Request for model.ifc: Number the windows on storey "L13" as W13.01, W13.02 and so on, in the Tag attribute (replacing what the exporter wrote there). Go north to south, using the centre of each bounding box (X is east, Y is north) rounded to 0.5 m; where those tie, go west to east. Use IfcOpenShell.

First a look at what the model holds.

```python
import ifcopenshell
import ifcopenshell.util.element
import ifcopenshell.util.placement

model = ifcopenshell.open("model.ifc")
print(model.schema)
storey = next(s for s in model.by_type("IfcBuildingStorey") if s.Name == "L13")
windows = [e for e in ifcopenshell.util.element.get_decomposition(storey) if e.is_a("IfcWindow")]
for e in sorted(windows, key=lambda e: e.id()):
    origin = ifcopenshell.util.placement.get_local_placement(e.ObjectPlacement)[:3, 3]
    print(e.id(), e.Tag, e.Name, origin.round(2) + 0.0, sep=" | ")
```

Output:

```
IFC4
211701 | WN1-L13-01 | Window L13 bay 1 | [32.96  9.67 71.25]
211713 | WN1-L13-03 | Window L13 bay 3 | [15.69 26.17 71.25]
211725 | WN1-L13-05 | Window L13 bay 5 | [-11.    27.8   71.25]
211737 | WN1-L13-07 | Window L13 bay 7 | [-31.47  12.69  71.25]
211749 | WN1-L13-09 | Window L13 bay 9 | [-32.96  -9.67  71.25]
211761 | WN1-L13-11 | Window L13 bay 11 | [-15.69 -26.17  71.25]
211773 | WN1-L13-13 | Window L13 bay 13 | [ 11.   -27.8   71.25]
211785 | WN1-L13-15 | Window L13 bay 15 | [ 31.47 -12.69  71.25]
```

```python
import ifcopenshell
import ifcopenshell.geom
import ifcopenshell.util.element
import ifcopenshell.util.shape

model = ifcopenshell.open("model.ifc")
settings = ifcopenshell.geom.settings()
settings.set("use-world-coords", True)


def centre(element):
    shape = ifcopenshell.geom.create_shape(settings, element)
    return ifcopenshell.util.shape.get_bbox_centroid(shape.geometry)


storey = next(s for s in model.by_type("IfcBuildingStorey") if s.Name == "L13")
windows = [e for e in ifcopenshell.util.element.get_decomposition(storey) if e.is_a("IfcWindow")]

# Insertion points can sit at a corner or the storey origin, so sort by the geometry (in metres).
centres = {e: centre(e) for e in windows}
windows.sort(key=lambda e: (-round(centres[e][1] / 0.5), centres[e][0]))

for i, e in enumerate(windows, start=1):
    number = f"W13.{i:02d}"
    e.Tag = number
    print(e.id(), number)

model.write("model-out.ifc")
```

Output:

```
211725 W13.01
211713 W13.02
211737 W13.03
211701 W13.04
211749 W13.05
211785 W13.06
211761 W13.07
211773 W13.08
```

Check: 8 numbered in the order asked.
